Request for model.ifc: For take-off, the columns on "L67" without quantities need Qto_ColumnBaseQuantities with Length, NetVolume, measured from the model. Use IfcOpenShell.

First a look at what the model holds.

```python
import ifcopenshell
import ifcopenshell.util.element
import ifcopenshell.util.unit

model = ifcopenshell.open("model.ifc")
print(model.schema)
for unit_type in ("LENGTHUNIT", "AREAUNIT", "VOLUMEUNIT"):
    print(unit_type, ifcopenshell.util.unit.calculate_unit_scale(model, unit_type))
storey = next(s for s in model.by_type("IfcBuildingStorey") if s.Name == "L67")
columns = [e for e in ifcopenshell.util.element.get_decomposition(storey) if e.is_a("IfcColumn")]
for e in sorted(columns, key=lambda e: e.id()):
    print(e.id(), e.is_a(), e.Name, list(ifcopenshell.util.element.get_psets(e, qtos_only=True)), sep=" | ")
```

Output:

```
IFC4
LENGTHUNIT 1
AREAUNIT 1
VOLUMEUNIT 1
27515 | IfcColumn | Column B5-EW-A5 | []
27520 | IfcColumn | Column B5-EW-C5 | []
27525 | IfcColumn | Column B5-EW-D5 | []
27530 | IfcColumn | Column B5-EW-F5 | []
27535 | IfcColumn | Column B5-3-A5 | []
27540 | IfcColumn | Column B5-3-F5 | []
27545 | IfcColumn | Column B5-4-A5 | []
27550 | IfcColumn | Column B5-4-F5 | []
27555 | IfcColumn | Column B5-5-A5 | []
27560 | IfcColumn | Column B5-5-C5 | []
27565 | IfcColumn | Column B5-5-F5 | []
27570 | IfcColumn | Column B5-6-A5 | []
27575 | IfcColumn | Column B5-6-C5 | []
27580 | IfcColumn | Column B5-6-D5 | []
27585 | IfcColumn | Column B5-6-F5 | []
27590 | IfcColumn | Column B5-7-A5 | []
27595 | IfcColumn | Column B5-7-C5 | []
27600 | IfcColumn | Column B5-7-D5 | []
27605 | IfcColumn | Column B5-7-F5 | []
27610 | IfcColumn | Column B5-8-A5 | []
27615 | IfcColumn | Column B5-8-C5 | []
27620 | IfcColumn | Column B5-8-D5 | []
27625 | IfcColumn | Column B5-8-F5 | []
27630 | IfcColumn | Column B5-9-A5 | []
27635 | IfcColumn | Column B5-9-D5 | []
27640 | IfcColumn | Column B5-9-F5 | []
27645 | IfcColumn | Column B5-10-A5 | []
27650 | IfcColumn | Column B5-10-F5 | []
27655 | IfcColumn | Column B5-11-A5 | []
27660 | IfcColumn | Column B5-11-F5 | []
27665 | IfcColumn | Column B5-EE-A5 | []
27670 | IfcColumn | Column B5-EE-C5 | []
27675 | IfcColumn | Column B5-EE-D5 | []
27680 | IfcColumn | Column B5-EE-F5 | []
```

```python
import ifcopenshell
import ifcopenshell.api.pset
import ifcopenshell.geom
import ifcopenshell.util.element
import ifcopenshell.util.shape
import ifcopenshell.util.unit

model = ifcopenshell.open("model.ifc")
unit_scale = ifcopenshell.util.unit.calculate_unit_scale(model)
volume_scale = ifcopenshell.util.unit.calculate_unit_scale(model, "VOLUMEUNIT")
settings = ifcopenshell.geom.settings()

storey = next(s for s in model.by_type("IfcBuildingStorey") if s.Name == "L67")
columns = [e for e in ifcopenshell.util.element.get_decomposition(storey) if e.is_a("IfcColumn")]

for e in sorted(columns, key=lambda e: e.id()):
    if ifcopenshell.util.element.get_psets(e, qtos_only=True, should_inherit=False):
        continue
    # Geometry comes back in metres, in the element's own axes.
    shape = ifcopenshell.geom.create_shape(settings, e)
    values = {
        "Length": ifcopenshell.util.shape.get_z(shape.geometry) / unit_scale,
        "NetVolume": ifcopenshell.util.shape.get_volume(shape.geometry) / volume_scale,
    }
    qto = ifcopenshell.api.pset.add_qto(model, product=e, name="Qto_ColumnBaseQuantities")
    ifcopenshell.api.pset.edit_qto(model, qto=qto, properties=values)
    print(e.id(), {k: round(v, 3) for k, v in values.items()})

model.write("model_v2.ifc")
```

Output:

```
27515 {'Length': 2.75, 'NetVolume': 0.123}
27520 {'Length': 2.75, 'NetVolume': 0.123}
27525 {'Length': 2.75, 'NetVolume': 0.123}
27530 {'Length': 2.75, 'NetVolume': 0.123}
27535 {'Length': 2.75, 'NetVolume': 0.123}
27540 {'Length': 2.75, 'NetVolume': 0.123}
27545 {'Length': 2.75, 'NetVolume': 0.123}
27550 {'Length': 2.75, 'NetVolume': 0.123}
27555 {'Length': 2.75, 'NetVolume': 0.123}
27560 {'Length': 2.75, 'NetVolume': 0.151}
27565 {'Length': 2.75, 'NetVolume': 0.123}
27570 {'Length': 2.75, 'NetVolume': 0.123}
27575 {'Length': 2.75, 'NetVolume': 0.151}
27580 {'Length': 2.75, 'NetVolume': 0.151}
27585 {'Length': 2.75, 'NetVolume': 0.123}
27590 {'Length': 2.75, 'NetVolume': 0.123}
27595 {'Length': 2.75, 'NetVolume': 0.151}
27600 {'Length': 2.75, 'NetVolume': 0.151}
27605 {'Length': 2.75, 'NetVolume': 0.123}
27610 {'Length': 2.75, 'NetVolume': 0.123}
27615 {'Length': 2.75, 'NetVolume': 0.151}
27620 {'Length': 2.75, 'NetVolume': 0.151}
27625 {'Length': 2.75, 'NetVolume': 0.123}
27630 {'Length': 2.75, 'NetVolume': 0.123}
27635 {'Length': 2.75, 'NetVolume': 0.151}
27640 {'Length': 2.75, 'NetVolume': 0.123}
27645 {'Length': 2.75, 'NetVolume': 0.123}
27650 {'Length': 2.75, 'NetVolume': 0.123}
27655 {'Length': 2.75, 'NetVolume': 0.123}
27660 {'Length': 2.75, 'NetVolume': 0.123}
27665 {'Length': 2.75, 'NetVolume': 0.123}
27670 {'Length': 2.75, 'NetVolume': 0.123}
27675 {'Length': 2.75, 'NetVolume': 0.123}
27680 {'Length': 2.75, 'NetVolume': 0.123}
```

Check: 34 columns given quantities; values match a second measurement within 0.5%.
